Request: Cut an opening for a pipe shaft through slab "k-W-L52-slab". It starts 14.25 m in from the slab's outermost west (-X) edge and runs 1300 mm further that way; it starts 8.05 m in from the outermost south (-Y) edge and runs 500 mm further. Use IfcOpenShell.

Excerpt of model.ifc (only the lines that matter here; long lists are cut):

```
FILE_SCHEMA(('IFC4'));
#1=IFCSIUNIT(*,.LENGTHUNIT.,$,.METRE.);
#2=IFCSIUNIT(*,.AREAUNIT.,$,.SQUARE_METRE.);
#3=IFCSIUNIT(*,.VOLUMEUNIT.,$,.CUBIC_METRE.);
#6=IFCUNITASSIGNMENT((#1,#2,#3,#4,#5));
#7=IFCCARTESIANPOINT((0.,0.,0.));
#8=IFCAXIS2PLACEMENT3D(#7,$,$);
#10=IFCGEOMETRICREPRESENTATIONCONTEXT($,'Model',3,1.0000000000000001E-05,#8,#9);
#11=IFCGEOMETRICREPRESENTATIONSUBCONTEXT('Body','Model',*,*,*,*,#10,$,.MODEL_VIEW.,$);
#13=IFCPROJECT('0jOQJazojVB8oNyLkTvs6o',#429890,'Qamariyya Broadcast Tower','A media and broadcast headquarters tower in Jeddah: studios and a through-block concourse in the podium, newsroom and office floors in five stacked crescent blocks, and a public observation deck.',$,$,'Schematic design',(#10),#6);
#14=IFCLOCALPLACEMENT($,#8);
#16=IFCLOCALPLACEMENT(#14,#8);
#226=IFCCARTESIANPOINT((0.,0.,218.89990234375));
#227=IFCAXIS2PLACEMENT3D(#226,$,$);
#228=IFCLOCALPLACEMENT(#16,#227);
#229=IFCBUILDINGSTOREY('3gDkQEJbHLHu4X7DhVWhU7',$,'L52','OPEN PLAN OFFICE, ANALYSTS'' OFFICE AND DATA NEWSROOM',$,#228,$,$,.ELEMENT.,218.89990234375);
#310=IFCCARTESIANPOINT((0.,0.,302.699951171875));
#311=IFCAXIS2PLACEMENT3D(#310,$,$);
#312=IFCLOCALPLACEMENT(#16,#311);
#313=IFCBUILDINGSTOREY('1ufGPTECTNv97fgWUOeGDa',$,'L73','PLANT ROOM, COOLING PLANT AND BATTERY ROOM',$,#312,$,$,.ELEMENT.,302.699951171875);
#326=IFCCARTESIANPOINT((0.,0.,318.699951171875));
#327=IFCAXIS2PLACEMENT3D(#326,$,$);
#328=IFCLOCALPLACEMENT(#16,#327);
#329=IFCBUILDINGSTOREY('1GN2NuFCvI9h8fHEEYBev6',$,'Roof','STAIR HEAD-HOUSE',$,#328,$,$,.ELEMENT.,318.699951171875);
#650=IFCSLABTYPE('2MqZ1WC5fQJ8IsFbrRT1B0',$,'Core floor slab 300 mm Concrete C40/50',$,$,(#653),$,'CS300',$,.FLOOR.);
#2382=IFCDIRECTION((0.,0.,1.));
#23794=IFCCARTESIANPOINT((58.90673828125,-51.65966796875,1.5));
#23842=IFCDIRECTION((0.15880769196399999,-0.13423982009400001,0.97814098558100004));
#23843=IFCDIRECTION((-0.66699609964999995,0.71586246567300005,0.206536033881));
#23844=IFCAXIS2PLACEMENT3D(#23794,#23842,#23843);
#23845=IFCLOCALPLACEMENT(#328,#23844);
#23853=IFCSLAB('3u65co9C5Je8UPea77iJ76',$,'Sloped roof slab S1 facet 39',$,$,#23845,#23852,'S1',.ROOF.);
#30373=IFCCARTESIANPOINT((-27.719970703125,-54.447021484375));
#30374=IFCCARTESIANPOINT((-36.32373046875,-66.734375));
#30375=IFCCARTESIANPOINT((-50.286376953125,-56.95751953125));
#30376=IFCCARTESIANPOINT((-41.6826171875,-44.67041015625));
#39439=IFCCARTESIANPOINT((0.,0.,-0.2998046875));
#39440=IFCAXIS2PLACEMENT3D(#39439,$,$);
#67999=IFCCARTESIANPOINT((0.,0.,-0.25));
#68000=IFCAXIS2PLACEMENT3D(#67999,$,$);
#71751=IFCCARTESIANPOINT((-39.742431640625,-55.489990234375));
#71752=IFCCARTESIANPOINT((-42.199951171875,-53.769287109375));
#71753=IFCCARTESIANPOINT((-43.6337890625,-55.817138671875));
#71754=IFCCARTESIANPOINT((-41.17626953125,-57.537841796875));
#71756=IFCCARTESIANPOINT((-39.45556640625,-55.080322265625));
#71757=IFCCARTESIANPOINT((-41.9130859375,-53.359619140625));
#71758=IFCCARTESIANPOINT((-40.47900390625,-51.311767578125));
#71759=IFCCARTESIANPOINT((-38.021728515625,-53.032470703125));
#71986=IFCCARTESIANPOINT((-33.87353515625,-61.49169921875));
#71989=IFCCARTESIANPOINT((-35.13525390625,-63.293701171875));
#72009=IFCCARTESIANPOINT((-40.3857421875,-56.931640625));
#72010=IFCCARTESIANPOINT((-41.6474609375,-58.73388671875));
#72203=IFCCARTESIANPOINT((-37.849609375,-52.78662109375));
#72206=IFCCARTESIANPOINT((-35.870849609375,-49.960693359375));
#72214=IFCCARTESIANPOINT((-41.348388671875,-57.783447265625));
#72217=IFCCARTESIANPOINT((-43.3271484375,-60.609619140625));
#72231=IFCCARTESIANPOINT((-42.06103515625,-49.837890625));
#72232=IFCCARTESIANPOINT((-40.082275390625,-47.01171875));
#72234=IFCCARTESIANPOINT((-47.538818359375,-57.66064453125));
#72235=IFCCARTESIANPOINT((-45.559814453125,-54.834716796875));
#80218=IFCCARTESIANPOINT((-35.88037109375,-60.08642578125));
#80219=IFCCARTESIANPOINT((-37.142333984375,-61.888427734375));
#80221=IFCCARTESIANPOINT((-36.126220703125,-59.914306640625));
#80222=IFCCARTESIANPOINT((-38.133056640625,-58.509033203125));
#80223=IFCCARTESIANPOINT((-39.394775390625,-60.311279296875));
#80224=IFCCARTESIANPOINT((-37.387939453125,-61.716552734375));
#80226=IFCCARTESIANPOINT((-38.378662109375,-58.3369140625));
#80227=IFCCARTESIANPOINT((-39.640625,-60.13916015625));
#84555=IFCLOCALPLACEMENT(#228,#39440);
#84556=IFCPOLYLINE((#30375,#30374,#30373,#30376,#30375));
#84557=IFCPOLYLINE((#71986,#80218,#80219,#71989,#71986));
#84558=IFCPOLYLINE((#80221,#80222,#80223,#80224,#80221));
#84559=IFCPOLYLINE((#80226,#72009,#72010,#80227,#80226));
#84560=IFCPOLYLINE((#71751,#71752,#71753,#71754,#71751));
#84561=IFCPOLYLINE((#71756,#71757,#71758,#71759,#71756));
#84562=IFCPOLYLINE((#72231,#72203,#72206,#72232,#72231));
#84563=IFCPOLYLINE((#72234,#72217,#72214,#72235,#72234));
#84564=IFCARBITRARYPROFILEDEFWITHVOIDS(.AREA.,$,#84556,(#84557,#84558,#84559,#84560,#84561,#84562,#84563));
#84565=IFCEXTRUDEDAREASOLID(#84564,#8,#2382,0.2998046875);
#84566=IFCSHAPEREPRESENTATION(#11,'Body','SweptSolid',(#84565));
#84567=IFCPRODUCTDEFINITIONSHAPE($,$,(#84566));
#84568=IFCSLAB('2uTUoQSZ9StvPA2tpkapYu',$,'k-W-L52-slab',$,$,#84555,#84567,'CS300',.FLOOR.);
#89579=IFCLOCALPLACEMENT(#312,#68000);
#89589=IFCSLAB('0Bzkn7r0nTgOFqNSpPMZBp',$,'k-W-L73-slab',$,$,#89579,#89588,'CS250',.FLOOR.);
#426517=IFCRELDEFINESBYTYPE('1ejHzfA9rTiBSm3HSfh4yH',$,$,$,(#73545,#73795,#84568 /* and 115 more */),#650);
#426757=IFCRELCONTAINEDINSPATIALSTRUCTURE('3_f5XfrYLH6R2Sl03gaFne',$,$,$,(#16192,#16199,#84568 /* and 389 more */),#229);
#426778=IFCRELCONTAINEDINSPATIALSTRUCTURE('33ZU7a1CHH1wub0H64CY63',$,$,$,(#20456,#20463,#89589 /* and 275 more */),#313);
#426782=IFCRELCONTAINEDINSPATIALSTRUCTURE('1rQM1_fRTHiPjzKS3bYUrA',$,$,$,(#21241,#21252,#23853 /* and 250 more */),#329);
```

```python
import numpy as np
import ifcopenshell
import ifcopenshell.api.feature
import ifcopenshell.api.geometry
import ifcopenshell.api.root
import ifcopenshell.geom
import ifcopenshell.util.placement
import ifcopenshell.util.representation
import ifcopenshell.util.shape
import ifcopenshell.util.unit

model = ifcopenshell.open("model.ifc")
unit_scale = ifcopenshell.util.unit.calculate_unit_scale(model)
settings = ifcopenshell.geom.settings()


def volume(element):
    """Net volume in cubic metres, openings subtracted."""
    shape = ifcopenshell.geom.create_shape(settings, element)
    return ifcopenshell.util.shape.get_volume(shape.geometry)


slab = model.by_guid("2uTUoQSZ9StvPA2tpkapYu")
before = volume(slab)

# Extent in the slab's own axes, in metres. The edges named are its -X and -Y sides.
slab_shape = ifcopenshell.geom.create_shape(settings, slab)
vertices = ifcopenshell.util.shape.get_vertices(slab_shape.geometry)
x_min, y_min, bottom = vertices.min(axis=0)
top = vertices[:, 2].max()

opening = ifcopenshell.api.root.create_entity(model, ifc_class="IfcOpeningElement", name="Pipe shaft opening", predefined_type="OPENING")
context = ifcopenshell.util.representation.get_context(model, "Model", "Body", "MODEL_VIEW")
width, depth = 1.3, 0.5
outline = [(0.0, 0.0), (width, 0.0), (width, depth), (0.0, depth), (0.0, 0.0)]
# Overshoot both faces by 50 mm so the cut is clean.
shape = ifcopenshell.api.geometry.add_slab_representation(
    model, context=context, depth=top - bottom + 0.1, polyline=outline
)
ifcopenshell.api.geometry.assign_representation(model, product=opening, representation=shape)

matrix = ifcopenshell.util.placement.get_local_placement(slab.ObjectPlacement)
matrix[:, 3] = matrix @ np.append(np.array([x_min + 14.25, y_min + 8.05, bottom - 0.05]) / unit_scale, 1.0)
ifcopenshell.api.geometry.edit_object_placement(model, product=opening, matrix=matrix, is_si=False)
ifcopenshell.api.feature.add_feature(model, feature=opening, element=slab)

after = volume(slab)

print(f"slab volume {before:.3f} -> {after:.3f} m3")

model.write("model_edited.ifc")
```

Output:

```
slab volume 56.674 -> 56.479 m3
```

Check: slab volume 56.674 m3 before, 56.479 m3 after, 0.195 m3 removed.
